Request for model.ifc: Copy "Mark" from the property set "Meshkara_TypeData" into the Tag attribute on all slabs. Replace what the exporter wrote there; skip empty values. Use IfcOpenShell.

First a look at what the model holds.

```python
import ifcopenshell
import ifcopenshell.util.element

model = ifcopenshell.open("model.ifc")
print(model.schema)
slabs = model.by_type("IfcSlab")
print(len(slabs), "slabs")
for e in slabs[:8]:
    source = ifcopenshell.util.element.get_pset(e, "Meshkara_TypeData", "Mark")
    target = e.Tag
    print(e.id(), repr(source), repr(target), sep=" | ")
```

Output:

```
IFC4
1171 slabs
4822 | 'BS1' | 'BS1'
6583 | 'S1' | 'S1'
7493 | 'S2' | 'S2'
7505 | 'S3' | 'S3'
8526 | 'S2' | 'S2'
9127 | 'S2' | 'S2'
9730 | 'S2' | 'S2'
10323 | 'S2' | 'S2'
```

```python
import ifcopenshell
import ifcopenshell.util.element

model = ifcopenshell.open("model.ifc")

count = 0
for e in model.by_type("IfcSlab"):
    value = ifcopenshell.util.element.get_pset(e, "Meshkara_TypeData", "Mark")
    current = e.Tag
    if not value or not value.strip() or current == value:
        continue
    e.Tag = value
    count += 1

print(count, "slabs updated")

model.write("model_updated.ifc")
```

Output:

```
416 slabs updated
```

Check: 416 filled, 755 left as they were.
